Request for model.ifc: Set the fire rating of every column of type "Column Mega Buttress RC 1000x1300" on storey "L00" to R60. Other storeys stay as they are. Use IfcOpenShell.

First a look at what the model holds.

```python
import ifcopenshell
import ifcopenshell.util.element

model = ifcopenshell.open("model.ifc")
print(model.schema)
storey = next(s for s in model.by_type("IfcBuildingStorey") if s.Name == "L00")
columns = [e for e in ifcopenshell.util.element.get_decomposition(storey) if e.is_a("IfcColumn")]
seen = {}
for e in columns:
    element_type = ifcopenshell.util.element.get_type(e)
    key = (element_type.Name if element_type != e and element_type else None, ifcopenshell.util.element.get_pset(e, "Pset_ColumnCommon", "FireRating"))
    seen[key] = seen.get(key, 0) + 1
for (name, value), count in sorted(seen.items(), key=str):
    print(count, "x", name, "|", value)
```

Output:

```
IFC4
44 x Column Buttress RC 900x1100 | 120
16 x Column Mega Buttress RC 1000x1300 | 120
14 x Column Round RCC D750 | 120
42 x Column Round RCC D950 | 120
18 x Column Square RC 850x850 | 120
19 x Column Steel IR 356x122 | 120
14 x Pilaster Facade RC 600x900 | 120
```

```python
import ifcopenshell
import ifcopenshell.api.pset
import ifcopenshell.util.element

model = ifcopenshell.open("model.ifc")

storey = next(s for s in model.by_type("IfcBuildingStorey") if s.Name == "L00")
columns = [e for e in ifcopenshell.util.element.get_decomposition(storey) if e.is_a("IfcColumn")]

count = 0
for e in columns:
    element_type = ifcopenshell.util.element.get_type(e)
    if element_type in (None, e) or element_type.Name != "Column Mega Buttress RC 1000x1300":
        continue
    # add_pset returns the element's existing set when there is one.
    pset = ifcopenshell.api.pset.add_pset(model, product=e, name="Pset_ColumnCommon")
    ifcopenshell.api.pset.edit_pset(model, pset=pset, properties={"FireRating": "R60"})
    count += 1

print(count, "columns updated")

model.write("model_rev.ifc")
```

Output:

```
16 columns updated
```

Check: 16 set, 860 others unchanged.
